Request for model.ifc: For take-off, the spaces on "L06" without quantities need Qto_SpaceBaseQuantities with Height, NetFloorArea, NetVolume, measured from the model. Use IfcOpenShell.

First a look at what the model holds.

```python
import ifcopenshell
import ifcopenshell.util.element
import ifcopenshell.util.unit

model = ifcopenshell.open("model.ifc")
print(model.schema)
for unit_type in ("LENGTHUNIT", "AREAUNIT", "VOLUMEUNIT"):
    print(unit_type, ifcopenshell.util.unit.calculate_unit_scale(model, unit_type))
storey = next(s for s in model.by_type("IfcBuildingStorey") if s.Name == "L06")
spaces = [e for e in ifcopenshell.util.element.get_decomposition(storey) if e.is_a("IfcSpace")]
for e in sorted(spaces, key=lambda e: e.id()):
    print(e.id(), e.is_a(), e.Name, list(ifcopenshell.util.element.get_psets(e, qtos_only=True)), sep=" | ")
```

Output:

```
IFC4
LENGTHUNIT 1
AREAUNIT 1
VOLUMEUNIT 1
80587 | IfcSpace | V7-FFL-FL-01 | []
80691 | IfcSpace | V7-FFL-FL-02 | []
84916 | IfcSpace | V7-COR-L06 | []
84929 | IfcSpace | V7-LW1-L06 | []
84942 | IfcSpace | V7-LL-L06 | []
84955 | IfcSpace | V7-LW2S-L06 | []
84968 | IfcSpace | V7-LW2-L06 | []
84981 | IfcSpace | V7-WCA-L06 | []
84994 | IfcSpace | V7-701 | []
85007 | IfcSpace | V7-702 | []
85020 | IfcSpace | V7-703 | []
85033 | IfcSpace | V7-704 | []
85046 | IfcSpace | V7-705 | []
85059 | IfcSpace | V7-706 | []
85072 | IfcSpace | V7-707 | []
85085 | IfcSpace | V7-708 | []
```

```python
import ifcopenshell
import ifcopenshell.api.pset
import ifcopenshell.geom
import ifcopenshell.util.element
import ifcopenshell.util.shape
import ifcopenshell.util.unit

model = ifcopenshell.open("model.ifc")
unit_scale = ifcopenshell.util.unit.calculate_unit_scale(model)
area_scale = ifcopenshell.util.unit.calculate_unit_scale(model, "AREAUNIT")
volume_scale = ifcopenshell.util.unit.calculate_unit_scale(model, "VOLUMEUNIT")
settings = ifcopenshell.geom.settings()

storey = next(s for s in model.by_type("IfcBuildingStorey") if s.Name == "L06")
spaces = [e for e in ifcopenshell.util.element.get_decomposition(storey) if e.is_a("IfcSpace")]

for e in sorted(spaces, key=lambda e: e.id()):
    if ifcopenshell.util.element.get_psets(e, qtos_only=True, should_inherit=False):
        continue
    # Geometry comes back in metres, in the element's own axes.
    shape = ifcopenshell.geom.create_shape(settings, e)
    values = {
        "Height": ifcopenshell.util.shape.get_z(shape.geometry) / unit_scale,
        "NetFloorArea": ifcopenshell.util.shape.get_footprint_area(shape.geometry) / area_scale,
        "NetVolume": ifcopenshell.util.shape.get_volume(shape.geometry) / volume_scale,
    }
    qto = ifcopenshell.api.pset.add_qto(model, product=e, name="Qto_SpaceBaseQuantities")
    ifcopenshell.api.pset.edit_qto(model, qto=qto, properties=values)
    print(e.id(), {k: round(v, 3) for k, v in values.items()})

model.write("model_edited.ifc")
```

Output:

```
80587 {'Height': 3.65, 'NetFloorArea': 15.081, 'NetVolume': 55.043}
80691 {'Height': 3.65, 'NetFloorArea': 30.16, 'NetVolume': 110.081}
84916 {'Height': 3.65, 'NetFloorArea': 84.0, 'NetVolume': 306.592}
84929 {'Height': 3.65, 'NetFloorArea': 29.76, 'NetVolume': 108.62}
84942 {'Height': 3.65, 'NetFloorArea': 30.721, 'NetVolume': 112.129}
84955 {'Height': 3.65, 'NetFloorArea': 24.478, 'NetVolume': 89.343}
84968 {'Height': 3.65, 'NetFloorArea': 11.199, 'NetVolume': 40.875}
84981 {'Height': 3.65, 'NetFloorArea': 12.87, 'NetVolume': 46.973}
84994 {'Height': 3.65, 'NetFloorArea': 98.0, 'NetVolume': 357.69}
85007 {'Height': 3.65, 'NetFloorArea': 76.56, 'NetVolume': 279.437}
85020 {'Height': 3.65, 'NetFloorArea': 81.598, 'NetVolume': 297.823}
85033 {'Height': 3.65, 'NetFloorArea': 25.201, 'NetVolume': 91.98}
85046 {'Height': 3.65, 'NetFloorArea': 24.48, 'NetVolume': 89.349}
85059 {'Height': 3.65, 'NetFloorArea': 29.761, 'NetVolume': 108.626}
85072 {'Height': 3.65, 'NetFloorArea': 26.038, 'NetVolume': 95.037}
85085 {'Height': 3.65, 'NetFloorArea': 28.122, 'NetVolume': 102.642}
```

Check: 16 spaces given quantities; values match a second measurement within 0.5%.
